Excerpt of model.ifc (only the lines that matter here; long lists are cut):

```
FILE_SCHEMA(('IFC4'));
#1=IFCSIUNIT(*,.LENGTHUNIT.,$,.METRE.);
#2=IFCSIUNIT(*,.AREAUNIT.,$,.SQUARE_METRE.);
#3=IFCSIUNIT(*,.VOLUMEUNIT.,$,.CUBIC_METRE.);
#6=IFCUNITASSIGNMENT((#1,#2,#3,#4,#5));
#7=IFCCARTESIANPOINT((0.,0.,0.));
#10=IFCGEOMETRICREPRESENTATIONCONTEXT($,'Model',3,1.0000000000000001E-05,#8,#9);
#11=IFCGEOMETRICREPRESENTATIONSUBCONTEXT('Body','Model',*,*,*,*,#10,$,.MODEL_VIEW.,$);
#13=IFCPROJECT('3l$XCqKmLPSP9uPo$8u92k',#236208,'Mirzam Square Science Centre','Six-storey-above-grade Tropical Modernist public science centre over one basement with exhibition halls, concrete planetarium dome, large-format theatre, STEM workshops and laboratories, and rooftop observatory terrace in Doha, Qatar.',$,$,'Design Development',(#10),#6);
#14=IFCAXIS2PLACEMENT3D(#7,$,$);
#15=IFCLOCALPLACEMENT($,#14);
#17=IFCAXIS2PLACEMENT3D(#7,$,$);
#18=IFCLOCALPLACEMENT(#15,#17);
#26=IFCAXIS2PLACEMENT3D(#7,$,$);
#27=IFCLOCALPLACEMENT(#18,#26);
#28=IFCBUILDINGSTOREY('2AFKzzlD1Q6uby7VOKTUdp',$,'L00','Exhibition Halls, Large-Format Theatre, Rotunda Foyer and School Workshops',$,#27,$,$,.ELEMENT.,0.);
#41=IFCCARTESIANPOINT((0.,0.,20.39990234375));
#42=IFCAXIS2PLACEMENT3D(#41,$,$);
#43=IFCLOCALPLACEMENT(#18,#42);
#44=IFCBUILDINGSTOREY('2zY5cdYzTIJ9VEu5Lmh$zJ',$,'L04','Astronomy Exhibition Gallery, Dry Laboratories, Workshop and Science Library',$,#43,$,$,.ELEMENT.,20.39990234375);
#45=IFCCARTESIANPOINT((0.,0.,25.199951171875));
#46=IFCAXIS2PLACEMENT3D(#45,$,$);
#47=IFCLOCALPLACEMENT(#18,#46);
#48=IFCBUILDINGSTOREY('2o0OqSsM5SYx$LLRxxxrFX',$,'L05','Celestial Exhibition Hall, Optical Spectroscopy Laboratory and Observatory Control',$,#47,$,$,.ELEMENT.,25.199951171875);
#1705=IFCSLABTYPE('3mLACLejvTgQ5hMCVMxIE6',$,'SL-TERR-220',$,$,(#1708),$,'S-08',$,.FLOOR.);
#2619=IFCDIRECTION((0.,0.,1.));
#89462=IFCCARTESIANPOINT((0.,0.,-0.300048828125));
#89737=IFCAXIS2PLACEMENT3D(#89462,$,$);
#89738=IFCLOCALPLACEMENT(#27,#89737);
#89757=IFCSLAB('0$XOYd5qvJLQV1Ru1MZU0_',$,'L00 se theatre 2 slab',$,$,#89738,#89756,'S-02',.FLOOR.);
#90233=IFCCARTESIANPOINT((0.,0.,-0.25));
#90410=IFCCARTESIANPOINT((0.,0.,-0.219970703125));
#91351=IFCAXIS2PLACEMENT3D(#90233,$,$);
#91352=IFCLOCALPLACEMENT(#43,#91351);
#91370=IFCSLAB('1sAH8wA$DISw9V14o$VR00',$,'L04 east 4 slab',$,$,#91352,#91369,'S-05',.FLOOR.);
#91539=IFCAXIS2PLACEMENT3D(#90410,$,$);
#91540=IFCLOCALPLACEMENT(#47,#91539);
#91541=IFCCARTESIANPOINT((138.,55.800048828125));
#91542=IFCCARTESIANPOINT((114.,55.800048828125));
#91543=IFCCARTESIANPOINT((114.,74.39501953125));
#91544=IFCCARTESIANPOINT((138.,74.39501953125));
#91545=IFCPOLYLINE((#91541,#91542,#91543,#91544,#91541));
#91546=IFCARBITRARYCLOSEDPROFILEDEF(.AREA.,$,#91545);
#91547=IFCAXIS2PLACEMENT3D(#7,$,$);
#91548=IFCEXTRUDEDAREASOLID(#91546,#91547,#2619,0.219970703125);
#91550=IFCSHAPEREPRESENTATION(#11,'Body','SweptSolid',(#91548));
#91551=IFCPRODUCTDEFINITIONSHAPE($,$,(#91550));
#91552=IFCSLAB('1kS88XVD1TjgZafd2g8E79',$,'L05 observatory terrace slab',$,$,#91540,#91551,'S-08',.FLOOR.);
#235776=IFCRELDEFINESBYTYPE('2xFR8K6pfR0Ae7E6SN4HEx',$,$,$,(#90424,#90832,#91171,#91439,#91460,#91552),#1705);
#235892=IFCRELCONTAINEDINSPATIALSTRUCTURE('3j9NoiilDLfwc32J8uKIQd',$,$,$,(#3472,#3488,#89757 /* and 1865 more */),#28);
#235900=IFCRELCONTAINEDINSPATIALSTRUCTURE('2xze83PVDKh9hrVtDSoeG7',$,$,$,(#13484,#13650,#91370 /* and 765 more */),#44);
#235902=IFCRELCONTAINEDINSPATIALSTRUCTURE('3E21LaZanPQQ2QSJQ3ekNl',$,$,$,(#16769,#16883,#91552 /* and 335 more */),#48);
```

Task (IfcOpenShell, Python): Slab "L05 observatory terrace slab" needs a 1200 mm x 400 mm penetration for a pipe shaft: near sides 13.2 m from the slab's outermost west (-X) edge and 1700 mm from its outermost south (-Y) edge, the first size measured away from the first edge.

```python
import numpy as np
import ifcopenshell
import ifcopenshell.api.feature
import ifcopenshell.api.geometry
import ifcopenshell.api.root
import ifcopenshell.geom
import ifcopenshell.util.placement
import ifcopenshell.util.representation
import ifcopenshell.util.shape
import ifcopenshell.util.unit

model = ifcopenshell.open("model.ifc")
unit_scale = ifcopenshell.util.unit.calculate_unit_scale(model)
settings = ifcopenshell.geom.settings()


def volume(element):
    """Net volume in cubic metres, openings subtracted."""
    shape = ifcopenshell.geom.create_shape(settings, element)
    return ifcopenshell.util.shape.get_volume(shape.geometry)


slab = model.by_id(91552)
before = volume(slab)

# Extent in the slab's own axes, in metres. The edges named are its -X and -Y sides.
slab_shape = ifcopenshell.geom.create_shape(settings, slab)
vertices = ifcopenshell.util.shape.get_vertices(slab_shape.geometry)
x_min, y_min, bottom = vertices.min(axis=0)
top = vertices[:, 2].max()

opening = ifcopenshell.api.root.create_entity(model, ifc_class="IfcOpeningElement", name="Pipe shaft opening", predefined_type="OPENING")
context = ifcopenshell.util.representation.get_context(model, "Model", "Body", "MODEL_VIEW")
width, depth = 1.2, 0.4
outline = [(0.0, 0.0), (width, 0.0), (width, depth), (0.0, depth), (0.0, 0.0)]
# Overshoot both faces by 50 mm so the cut is clean.
shape = ifcopenshell.api.geometry.add_slab_representation(
    model, context=context, depth=top - bottom + 0.1, polyline=outline
)
ifcopenshell.api.geometry.assign_representation(model, product=opening, representation=shape)

matrix = ifcopenshell.util.placement.get_local_placement(slab.ObjectPlacement)
matrix[:, 3] = matrix @ np.append(np.array([x_min + 13.2, y_min + 1.7, bottom - 0.05]) / unit_scale, 1.0)
ifcopenshell.api.geometry.edit_object_placement(model, product=opening, matrix=matrix, is_si=False)
ifcopenshell.api.feature.add_feature(model, feature=opening, element=slab)

after = volume(slab)

print(f"slab volume {before:.3f} -> {after:.3f} m3")

model.write("model_edited.ifc")
```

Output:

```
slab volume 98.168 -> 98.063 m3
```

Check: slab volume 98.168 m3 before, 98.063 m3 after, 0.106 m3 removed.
